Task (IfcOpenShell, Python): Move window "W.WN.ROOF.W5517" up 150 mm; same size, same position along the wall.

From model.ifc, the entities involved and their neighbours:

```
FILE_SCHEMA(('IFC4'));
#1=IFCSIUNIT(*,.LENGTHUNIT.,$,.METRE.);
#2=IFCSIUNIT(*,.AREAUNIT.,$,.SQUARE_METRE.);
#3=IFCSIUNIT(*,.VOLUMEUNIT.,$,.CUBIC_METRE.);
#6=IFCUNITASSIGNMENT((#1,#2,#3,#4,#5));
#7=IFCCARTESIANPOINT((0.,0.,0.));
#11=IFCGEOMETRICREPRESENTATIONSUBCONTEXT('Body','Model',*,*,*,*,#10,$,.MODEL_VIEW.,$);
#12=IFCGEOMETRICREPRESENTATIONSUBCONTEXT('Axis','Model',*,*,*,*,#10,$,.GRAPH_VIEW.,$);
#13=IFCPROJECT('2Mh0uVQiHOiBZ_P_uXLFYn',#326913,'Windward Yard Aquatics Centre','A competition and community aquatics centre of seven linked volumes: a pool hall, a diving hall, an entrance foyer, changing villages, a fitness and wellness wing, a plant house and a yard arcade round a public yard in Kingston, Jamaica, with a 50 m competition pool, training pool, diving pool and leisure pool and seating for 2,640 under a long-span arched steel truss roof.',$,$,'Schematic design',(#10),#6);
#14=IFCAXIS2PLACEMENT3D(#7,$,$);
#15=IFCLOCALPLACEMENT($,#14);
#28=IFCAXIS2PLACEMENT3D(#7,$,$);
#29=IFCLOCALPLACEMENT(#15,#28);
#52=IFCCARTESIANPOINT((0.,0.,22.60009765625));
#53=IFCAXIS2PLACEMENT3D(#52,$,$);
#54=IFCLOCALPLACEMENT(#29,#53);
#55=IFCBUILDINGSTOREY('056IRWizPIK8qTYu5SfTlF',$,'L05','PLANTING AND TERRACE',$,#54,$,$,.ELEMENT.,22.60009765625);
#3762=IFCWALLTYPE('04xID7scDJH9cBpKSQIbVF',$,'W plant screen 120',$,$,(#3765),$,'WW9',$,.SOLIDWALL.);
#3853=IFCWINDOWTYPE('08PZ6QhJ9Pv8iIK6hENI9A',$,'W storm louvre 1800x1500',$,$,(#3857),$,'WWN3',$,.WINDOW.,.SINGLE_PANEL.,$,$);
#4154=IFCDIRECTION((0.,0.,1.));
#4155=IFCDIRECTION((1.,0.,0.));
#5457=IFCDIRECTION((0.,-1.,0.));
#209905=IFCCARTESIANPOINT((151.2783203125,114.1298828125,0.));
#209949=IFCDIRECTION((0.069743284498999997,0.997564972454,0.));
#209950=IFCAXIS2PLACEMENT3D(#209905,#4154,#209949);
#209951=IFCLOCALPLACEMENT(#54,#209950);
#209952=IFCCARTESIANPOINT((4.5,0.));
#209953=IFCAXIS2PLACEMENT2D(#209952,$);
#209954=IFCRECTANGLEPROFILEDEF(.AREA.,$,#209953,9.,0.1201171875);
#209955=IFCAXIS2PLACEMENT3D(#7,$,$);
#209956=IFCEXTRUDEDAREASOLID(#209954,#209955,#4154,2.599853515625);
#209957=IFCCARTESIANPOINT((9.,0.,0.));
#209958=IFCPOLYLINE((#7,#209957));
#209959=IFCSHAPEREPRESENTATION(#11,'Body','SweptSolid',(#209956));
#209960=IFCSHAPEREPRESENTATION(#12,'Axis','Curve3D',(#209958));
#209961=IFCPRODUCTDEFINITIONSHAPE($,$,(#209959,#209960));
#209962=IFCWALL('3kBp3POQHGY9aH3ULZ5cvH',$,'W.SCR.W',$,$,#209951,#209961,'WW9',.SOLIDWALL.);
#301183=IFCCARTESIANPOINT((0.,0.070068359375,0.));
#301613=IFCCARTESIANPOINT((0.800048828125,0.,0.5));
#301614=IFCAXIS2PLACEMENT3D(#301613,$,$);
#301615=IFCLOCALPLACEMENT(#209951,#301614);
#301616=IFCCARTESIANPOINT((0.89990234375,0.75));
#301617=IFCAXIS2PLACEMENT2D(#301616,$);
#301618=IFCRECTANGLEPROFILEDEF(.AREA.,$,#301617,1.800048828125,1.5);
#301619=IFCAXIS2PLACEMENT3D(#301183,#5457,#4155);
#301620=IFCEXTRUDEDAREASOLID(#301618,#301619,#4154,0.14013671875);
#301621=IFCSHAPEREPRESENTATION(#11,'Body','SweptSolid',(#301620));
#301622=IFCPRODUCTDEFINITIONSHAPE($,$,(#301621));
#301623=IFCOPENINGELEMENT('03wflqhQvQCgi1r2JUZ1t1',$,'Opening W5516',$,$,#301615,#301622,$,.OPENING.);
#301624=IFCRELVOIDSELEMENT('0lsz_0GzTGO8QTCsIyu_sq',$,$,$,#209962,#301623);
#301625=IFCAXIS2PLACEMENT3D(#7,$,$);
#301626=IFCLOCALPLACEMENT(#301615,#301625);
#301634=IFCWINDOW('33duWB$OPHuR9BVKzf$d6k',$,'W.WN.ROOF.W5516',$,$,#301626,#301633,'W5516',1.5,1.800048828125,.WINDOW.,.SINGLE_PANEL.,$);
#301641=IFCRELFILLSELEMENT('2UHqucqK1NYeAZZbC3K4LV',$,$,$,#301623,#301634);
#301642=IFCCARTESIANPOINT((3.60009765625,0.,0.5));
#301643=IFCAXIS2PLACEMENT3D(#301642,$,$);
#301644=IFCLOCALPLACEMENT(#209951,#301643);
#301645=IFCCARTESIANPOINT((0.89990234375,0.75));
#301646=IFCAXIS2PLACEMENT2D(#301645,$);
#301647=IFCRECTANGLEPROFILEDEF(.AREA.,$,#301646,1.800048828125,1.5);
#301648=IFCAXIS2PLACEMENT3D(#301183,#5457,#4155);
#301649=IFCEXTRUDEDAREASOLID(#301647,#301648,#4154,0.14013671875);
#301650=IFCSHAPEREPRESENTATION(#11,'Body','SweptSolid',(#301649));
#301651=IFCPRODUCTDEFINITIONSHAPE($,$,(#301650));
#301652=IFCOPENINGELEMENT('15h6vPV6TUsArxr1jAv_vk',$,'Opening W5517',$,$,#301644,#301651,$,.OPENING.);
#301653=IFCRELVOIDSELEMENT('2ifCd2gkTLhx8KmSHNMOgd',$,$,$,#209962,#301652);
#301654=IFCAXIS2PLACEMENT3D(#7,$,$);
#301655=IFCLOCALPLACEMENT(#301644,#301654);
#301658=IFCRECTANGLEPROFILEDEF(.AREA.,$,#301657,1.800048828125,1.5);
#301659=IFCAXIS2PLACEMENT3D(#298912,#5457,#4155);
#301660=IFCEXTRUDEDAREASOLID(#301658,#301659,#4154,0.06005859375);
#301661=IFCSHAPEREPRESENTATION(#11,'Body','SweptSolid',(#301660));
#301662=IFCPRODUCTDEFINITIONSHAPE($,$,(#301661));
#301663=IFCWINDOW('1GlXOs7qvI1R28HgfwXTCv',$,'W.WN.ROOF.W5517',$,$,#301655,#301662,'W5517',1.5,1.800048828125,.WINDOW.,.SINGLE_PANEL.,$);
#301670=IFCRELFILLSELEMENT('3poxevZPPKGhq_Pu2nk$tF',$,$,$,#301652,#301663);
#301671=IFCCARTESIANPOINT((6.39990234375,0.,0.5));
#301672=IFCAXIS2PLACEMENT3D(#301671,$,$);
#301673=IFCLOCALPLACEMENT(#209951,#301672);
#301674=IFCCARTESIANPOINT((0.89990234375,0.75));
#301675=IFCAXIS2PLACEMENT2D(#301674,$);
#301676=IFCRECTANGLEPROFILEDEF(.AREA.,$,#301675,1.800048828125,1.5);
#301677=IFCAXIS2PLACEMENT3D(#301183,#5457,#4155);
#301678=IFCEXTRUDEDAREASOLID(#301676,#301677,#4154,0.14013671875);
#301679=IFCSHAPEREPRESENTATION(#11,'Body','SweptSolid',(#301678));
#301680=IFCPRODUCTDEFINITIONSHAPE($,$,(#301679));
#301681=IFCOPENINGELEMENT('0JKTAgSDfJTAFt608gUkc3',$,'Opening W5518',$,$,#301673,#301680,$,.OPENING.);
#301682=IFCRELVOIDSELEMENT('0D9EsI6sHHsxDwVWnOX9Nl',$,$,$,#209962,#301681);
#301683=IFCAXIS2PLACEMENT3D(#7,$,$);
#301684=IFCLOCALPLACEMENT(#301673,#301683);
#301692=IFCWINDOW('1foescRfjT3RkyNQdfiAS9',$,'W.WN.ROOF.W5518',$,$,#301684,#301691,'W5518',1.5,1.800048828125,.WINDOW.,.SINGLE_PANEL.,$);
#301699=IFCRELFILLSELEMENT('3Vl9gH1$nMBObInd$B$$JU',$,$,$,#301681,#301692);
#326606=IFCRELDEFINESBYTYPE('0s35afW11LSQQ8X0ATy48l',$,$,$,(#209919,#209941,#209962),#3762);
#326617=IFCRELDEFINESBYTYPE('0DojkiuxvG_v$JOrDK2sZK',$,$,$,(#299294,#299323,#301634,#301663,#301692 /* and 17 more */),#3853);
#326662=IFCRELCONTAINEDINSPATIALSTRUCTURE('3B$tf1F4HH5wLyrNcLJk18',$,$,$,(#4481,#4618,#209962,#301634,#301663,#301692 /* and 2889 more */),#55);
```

```python
import numpy as np
import ifcopenshell
import ifcopenshell.api.geometry
import ifcopenshell.util.placement
import ifcopenshell.util.unit

model = ifcopenshell.open("model.ifc")
unit_scale = ifcopenshell.util.unit.calculate_unit_scale(model)

window = model.by_id(301663)
opening = window.FillsVoids[0].RelatingOpeningElement
dz = 0.15

shift = np.array([0.0, 0.0, dz])
# The window is placed relative to its opening, so it follows when the opening moves.
matrix = ifcopenshell.util.placement.get_local_placement(opening.ObjectPlacement)
matrix[:3, 3] += shift
ifcopenshell.api.geometry.edit_object_placement(
    model, product=opening, matrix=matrix, is_si=False, should_transform_children=True
)

print(f"moved by {dz * unit_scale:+.3f} m")

model.write("model-out.ifc")
```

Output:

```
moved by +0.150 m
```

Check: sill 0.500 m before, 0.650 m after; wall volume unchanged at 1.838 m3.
